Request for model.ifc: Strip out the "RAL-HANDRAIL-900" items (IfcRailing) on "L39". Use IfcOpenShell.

First a look at what the model holds.

```python
import ifcopenshell
import ifcopenshell.util.element

model = ifcopenshell.open("model.ifc")
print(model.schema)
storey = next(s for s in model.by_type("IfcBuildingStorey") if s.Name == "L39")
railings = [e for e in ifcopenshell.util.element.get_decomposition(storey) if e.is_a("IfcRailing")]
seen = {}
for e in railings:
    element_type = ifcopenshell.util.element.get_type(e)
    name = element_type.Name if element_type not in (None, e) else None
    seen[name] = seen.get(name, 0) + 1
for name, count in sorted(seen.items(), key=str):
    print(count, "x", name)
```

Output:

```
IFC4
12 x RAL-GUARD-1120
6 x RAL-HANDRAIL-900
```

```python
import ifcopenshell
import ifcopenshell.api.root
import ifcopenshell.util.element

model = ifcopenshell.open("model.ifc")

storey = next(s for s in model.by_type("IfcBuildingStorey") if s.Name == "L39")
railings = [e for e in ifcopenshell.util.element.get_decomposition(storey) if e.is_a("IfcRailing")]
targets = [e for e in railings if (t := ifcopenshell.util.element.get_type(e)) not in (None, e) and t.Name == "RAL-HANDRAIL-900"]

for e in targets:
    ifcopenshell.api.root.remove_product(model, product=e)
print(len(targets), "removed")

model.write("model_rev.ifc")
```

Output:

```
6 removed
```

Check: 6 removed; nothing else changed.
